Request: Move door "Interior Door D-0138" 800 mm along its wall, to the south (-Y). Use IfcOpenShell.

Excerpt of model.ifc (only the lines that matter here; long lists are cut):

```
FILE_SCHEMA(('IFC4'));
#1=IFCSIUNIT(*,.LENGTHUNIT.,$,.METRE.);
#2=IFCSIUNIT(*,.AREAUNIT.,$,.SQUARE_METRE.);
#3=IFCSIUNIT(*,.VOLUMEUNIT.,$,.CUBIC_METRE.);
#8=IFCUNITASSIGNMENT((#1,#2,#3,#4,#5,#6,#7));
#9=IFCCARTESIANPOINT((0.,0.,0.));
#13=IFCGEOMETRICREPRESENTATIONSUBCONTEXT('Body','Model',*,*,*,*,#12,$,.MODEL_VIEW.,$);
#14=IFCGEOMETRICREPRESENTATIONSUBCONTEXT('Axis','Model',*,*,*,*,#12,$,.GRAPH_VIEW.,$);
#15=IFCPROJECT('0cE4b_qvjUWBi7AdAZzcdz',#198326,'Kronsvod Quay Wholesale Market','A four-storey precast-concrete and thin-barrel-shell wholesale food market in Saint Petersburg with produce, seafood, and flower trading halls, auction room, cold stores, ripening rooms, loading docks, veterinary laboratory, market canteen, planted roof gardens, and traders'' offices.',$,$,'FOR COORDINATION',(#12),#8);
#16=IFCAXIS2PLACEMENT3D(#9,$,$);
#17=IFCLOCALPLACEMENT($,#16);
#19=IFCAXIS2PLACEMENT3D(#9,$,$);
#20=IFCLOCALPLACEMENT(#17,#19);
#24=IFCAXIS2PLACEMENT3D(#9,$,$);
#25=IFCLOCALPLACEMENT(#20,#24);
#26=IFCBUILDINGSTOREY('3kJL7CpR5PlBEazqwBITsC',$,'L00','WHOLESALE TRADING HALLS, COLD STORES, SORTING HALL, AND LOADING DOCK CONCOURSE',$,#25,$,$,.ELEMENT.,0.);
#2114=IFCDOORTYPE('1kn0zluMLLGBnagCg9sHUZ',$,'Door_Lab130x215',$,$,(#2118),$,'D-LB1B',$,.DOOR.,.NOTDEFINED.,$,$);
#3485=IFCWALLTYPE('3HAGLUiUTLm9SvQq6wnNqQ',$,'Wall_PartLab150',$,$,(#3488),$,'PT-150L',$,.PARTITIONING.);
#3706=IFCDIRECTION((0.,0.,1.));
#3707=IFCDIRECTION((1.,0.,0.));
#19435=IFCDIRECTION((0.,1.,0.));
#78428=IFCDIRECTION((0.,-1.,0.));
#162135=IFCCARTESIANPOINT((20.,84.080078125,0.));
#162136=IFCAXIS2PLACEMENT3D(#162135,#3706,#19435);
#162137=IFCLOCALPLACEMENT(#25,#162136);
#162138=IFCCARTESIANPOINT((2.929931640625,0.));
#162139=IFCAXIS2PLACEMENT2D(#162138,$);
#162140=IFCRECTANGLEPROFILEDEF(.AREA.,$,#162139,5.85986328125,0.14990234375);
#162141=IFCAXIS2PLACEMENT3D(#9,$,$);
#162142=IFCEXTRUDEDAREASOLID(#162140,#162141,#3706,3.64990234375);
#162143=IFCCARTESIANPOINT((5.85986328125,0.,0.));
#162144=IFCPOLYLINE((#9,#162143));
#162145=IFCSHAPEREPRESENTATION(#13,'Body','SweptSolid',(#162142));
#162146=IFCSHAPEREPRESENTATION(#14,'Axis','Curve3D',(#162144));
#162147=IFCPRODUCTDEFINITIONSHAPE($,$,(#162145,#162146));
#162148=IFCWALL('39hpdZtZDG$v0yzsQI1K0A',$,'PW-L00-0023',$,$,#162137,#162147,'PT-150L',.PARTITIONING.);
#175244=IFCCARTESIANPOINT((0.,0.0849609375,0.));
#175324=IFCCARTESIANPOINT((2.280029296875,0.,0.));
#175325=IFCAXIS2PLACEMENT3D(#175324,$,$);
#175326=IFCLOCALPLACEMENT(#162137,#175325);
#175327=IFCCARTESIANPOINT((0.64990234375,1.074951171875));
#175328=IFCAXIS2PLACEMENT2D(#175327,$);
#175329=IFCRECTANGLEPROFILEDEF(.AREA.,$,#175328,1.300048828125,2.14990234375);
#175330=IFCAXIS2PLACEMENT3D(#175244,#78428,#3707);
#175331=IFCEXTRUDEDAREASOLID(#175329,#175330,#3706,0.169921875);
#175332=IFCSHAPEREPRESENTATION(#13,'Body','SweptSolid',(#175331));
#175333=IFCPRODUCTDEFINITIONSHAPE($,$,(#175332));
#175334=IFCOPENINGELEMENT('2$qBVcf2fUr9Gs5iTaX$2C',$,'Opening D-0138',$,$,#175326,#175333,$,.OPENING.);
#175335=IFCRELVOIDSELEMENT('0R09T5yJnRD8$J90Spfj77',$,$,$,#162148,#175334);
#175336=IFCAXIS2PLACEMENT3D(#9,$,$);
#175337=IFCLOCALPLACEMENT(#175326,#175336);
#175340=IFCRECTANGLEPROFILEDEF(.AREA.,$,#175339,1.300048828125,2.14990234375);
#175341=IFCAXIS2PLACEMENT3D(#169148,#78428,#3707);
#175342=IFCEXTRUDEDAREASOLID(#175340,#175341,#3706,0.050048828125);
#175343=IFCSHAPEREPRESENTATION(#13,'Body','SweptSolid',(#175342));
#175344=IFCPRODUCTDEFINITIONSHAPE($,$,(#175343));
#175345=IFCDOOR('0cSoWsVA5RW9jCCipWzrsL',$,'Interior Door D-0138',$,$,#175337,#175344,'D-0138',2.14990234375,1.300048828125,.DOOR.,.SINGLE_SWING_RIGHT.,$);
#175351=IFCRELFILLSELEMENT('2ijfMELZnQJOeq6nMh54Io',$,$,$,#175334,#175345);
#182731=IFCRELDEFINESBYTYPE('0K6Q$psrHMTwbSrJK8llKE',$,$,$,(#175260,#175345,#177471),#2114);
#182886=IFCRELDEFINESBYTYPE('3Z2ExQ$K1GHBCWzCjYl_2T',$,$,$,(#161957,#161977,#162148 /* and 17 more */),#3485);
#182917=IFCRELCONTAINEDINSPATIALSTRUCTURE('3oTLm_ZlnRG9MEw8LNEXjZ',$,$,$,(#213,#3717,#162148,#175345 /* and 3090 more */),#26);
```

```python
import ifcopenshell
import ifcopenshell.api.geometry
import ifcopenshell.util.placement
import ifcopenshell.util.unit

model = ifcopenshell.open("model.ifc")
unit_scale = ifcopenshell.util.unit.calculate_unit_scale(model)

door = model.by_guid("0cSoWsVA5RW9jCCipWzrsL")
opening = door.FillsVoids[0].RelatingOpeningElement
wall = opening.VoidsElements[0].RelatingBuildingElement

wall_matrix = ifcopenshell.util.placement.get_local_placement(wall.ObjectPlacement)
shift = wall_matrix[:3, 0] * -0.8 / unit_scale
before = ifcopenshell.util.placement.get_local_placement(door.ObjectPlacement)[:3, 3].copy()

# The door is placed relative to its opening, so it follows when the opening moves.
matrix = ifcopenshell.util.placement.get_local_placement(opening.ObjectPlacement)
matrix[:3, 3] += shift
ifcopenshell.api.geometry.edit_object_placement(
    model, product=opening, matrix=matrix, is_si=False, should_transform_children=True
)

after = ifcopenshell.util.placement.get_local_placement(door.ObjectPlacement)[:3, 3]
print("door moved by", (after - before).round(3) + 0.0)

model.write("model_edited.ifc")
```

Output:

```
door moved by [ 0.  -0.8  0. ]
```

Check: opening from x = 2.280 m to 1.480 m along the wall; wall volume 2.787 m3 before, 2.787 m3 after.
